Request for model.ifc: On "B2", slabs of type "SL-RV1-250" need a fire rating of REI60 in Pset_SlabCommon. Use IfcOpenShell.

First a look at what the model holds.

```python
import ifcopenshell
import ifcopenshell.util.element

model = ifcopenshell.open("model.ifc")
print(model.schema)
storey = next(s for s in model.by_type("IfcBuildingStorey") if s.Name == "B2")
slabs = [e for e in ifcopenshell.util.element.get_decomposition(storey) if e.is_a("IfcSlab")]
seen = {}
for e in slabs:
    element_type = ifcopenshell.util.element.get_type(e)
    key = (element_type.Name if element_type != e and element_type else None, ifcopenshell.util.element.get_pset(e, "Pset_SlabCommon", "FireRating"))
    seen[key] = seen.get(key, 0) + 1
for (name, value), count in sorted(seen.items(), key=str):
    print(count, "x", name, "|", value)
```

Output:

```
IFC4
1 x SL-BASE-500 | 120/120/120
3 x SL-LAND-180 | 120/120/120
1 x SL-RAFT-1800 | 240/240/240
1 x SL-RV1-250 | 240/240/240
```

```python
import ifcopenshell
import ifcopenshell.api.pset
import ifcopenshell.util.element

model = ifcopenshell.open("model.ifc")

storey = next(s for s in model.by_type("IfcBuildingStorey") if s.Name == "B2")
slabs = [e for e in ifcopenshell.util.element.get_decomposition(storey) if e.is_a("IfcSlab")]

count = 0
for e in slabs:
    element_type = ifcopenshell.util.element.get_type(e)
    if element_type in (None, e) or element_type.Name != "SL-RV1-250":
        continue
    # add_pset returns the element's existing set when there is one.
    pset = ifcopenshell.api.pset.add_pset(model, product=e, name="Pset_SlabCommon")
    ifcopenshell.api.pset.edit_pset(model, pset=pset, properties={"FireRating": "REI60"})
    count += 1

print(count, "slabs updated")

model.write("model_rev.ifc")
```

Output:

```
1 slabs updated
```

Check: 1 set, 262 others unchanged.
